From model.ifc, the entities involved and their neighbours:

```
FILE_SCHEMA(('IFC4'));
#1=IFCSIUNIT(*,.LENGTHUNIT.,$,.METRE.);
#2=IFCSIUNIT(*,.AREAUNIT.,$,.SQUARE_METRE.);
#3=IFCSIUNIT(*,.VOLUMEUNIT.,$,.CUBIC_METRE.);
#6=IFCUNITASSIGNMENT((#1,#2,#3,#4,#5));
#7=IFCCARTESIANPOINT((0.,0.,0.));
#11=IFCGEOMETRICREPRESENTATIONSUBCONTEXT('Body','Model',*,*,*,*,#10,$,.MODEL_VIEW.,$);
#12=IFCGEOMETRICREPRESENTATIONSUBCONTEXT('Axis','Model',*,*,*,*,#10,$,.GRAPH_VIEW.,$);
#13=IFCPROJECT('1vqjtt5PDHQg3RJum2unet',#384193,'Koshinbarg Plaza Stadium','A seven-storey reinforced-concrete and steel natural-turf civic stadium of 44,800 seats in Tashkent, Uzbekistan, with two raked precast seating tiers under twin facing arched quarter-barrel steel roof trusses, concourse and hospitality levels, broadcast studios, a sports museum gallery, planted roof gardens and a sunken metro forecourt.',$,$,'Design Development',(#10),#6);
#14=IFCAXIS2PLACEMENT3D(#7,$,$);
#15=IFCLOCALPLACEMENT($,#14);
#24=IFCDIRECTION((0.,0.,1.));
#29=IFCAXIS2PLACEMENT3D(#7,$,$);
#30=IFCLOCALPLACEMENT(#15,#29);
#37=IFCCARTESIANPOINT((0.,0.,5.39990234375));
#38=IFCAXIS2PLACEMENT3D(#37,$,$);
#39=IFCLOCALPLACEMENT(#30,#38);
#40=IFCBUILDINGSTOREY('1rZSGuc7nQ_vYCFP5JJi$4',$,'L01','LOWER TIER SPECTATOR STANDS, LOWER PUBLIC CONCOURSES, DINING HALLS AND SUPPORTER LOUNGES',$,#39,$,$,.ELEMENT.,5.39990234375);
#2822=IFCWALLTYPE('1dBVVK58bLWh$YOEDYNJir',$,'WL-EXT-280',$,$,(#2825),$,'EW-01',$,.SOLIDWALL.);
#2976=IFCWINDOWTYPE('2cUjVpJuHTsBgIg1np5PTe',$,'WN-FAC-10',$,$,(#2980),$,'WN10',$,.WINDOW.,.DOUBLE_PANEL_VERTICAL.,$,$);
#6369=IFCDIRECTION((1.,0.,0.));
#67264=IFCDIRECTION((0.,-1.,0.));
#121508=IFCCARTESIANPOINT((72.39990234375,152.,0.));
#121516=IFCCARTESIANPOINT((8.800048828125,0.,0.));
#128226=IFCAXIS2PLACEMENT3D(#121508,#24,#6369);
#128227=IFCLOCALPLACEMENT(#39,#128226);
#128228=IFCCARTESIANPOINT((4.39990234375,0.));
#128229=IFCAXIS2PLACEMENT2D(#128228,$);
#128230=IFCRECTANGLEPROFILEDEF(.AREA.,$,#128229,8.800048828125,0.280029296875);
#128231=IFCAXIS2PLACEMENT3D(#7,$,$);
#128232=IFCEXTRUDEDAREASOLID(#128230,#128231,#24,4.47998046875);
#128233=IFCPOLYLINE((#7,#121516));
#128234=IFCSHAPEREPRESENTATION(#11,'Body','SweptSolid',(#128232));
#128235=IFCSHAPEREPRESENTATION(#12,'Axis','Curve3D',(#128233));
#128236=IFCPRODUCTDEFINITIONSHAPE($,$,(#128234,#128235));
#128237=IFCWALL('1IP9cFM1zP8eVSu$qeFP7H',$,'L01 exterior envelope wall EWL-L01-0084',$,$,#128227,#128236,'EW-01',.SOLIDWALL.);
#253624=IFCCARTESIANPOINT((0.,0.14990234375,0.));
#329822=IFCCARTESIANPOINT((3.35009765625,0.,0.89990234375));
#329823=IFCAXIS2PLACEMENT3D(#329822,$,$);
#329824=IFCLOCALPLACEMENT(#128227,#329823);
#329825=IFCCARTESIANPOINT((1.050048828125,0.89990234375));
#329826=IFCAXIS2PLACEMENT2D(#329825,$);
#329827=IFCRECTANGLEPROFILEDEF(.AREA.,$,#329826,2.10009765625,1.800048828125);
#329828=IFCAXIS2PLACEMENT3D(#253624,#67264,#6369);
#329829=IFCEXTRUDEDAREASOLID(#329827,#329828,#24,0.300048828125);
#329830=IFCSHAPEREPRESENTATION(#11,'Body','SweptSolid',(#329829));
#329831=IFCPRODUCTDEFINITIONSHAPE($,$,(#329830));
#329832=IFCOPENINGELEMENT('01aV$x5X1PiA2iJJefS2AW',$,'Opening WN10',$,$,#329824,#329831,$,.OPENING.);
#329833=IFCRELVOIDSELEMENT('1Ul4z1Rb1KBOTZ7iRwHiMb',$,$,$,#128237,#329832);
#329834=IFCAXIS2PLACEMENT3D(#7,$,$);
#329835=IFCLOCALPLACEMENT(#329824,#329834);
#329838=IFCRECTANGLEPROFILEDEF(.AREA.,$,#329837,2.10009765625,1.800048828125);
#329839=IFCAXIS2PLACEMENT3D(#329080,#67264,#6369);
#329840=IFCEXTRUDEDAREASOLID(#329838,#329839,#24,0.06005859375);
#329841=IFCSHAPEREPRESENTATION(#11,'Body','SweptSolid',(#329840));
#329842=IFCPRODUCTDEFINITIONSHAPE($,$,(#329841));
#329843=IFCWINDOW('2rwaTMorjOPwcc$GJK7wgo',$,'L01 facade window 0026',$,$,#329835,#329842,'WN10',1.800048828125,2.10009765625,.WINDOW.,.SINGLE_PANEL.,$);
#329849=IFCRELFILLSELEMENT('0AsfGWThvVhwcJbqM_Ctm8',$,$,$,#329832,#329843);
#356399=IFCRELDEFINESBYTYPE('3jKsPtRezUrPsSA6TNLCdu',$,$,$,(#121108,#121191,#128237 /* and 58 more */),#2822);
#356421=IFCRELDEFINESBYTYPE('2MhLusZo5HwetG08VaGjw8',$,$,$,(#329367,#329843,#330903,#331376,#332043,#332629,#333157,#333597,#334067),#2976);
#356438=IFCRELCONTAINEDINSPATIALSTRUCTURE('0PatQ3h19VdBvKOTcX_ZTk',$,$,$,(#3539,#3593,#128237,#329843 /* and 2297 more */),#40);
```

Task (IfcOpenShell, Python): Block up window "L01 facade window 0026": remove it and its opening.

```python
import ifcopenshell
import ifcopenshell.api.feature
import ifcopenshell.api.root
import ifcopenshell.geom
import ifcopenshell.util.shape

model = ifcopenshell.open("model.ifc")
settings = ifcopenshell.geom.settings()


def volume(element):
    """Net volume in cubic metres, openings subtracted."""
    shape = ifcopenshell.geom.create_shape(settings, element)
    return ifcopenshell.util.shape.get_volume(shape.geometry)


window = model.by_guid("2rwaTMorjOPwcc$GJK7wgo")
opening = window.FillsVoids[0].RelatingOpeningElement
wall = opening.VoidsElements[0].RelatingBuildingElement
before = volume(wall)

ifcopenshell.api.root.remove_product(model, product=window)
ifcopenshell.api.feature.remove_feature(model, feature=opening)

after = volume(wall)

print(f"wall volume {before:.3f} -> {after:.3f} m3")

model.write("model_edited.ifc")
```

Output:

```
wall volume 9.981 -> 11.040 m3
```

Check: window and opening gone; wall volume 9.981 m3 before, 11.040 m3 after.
